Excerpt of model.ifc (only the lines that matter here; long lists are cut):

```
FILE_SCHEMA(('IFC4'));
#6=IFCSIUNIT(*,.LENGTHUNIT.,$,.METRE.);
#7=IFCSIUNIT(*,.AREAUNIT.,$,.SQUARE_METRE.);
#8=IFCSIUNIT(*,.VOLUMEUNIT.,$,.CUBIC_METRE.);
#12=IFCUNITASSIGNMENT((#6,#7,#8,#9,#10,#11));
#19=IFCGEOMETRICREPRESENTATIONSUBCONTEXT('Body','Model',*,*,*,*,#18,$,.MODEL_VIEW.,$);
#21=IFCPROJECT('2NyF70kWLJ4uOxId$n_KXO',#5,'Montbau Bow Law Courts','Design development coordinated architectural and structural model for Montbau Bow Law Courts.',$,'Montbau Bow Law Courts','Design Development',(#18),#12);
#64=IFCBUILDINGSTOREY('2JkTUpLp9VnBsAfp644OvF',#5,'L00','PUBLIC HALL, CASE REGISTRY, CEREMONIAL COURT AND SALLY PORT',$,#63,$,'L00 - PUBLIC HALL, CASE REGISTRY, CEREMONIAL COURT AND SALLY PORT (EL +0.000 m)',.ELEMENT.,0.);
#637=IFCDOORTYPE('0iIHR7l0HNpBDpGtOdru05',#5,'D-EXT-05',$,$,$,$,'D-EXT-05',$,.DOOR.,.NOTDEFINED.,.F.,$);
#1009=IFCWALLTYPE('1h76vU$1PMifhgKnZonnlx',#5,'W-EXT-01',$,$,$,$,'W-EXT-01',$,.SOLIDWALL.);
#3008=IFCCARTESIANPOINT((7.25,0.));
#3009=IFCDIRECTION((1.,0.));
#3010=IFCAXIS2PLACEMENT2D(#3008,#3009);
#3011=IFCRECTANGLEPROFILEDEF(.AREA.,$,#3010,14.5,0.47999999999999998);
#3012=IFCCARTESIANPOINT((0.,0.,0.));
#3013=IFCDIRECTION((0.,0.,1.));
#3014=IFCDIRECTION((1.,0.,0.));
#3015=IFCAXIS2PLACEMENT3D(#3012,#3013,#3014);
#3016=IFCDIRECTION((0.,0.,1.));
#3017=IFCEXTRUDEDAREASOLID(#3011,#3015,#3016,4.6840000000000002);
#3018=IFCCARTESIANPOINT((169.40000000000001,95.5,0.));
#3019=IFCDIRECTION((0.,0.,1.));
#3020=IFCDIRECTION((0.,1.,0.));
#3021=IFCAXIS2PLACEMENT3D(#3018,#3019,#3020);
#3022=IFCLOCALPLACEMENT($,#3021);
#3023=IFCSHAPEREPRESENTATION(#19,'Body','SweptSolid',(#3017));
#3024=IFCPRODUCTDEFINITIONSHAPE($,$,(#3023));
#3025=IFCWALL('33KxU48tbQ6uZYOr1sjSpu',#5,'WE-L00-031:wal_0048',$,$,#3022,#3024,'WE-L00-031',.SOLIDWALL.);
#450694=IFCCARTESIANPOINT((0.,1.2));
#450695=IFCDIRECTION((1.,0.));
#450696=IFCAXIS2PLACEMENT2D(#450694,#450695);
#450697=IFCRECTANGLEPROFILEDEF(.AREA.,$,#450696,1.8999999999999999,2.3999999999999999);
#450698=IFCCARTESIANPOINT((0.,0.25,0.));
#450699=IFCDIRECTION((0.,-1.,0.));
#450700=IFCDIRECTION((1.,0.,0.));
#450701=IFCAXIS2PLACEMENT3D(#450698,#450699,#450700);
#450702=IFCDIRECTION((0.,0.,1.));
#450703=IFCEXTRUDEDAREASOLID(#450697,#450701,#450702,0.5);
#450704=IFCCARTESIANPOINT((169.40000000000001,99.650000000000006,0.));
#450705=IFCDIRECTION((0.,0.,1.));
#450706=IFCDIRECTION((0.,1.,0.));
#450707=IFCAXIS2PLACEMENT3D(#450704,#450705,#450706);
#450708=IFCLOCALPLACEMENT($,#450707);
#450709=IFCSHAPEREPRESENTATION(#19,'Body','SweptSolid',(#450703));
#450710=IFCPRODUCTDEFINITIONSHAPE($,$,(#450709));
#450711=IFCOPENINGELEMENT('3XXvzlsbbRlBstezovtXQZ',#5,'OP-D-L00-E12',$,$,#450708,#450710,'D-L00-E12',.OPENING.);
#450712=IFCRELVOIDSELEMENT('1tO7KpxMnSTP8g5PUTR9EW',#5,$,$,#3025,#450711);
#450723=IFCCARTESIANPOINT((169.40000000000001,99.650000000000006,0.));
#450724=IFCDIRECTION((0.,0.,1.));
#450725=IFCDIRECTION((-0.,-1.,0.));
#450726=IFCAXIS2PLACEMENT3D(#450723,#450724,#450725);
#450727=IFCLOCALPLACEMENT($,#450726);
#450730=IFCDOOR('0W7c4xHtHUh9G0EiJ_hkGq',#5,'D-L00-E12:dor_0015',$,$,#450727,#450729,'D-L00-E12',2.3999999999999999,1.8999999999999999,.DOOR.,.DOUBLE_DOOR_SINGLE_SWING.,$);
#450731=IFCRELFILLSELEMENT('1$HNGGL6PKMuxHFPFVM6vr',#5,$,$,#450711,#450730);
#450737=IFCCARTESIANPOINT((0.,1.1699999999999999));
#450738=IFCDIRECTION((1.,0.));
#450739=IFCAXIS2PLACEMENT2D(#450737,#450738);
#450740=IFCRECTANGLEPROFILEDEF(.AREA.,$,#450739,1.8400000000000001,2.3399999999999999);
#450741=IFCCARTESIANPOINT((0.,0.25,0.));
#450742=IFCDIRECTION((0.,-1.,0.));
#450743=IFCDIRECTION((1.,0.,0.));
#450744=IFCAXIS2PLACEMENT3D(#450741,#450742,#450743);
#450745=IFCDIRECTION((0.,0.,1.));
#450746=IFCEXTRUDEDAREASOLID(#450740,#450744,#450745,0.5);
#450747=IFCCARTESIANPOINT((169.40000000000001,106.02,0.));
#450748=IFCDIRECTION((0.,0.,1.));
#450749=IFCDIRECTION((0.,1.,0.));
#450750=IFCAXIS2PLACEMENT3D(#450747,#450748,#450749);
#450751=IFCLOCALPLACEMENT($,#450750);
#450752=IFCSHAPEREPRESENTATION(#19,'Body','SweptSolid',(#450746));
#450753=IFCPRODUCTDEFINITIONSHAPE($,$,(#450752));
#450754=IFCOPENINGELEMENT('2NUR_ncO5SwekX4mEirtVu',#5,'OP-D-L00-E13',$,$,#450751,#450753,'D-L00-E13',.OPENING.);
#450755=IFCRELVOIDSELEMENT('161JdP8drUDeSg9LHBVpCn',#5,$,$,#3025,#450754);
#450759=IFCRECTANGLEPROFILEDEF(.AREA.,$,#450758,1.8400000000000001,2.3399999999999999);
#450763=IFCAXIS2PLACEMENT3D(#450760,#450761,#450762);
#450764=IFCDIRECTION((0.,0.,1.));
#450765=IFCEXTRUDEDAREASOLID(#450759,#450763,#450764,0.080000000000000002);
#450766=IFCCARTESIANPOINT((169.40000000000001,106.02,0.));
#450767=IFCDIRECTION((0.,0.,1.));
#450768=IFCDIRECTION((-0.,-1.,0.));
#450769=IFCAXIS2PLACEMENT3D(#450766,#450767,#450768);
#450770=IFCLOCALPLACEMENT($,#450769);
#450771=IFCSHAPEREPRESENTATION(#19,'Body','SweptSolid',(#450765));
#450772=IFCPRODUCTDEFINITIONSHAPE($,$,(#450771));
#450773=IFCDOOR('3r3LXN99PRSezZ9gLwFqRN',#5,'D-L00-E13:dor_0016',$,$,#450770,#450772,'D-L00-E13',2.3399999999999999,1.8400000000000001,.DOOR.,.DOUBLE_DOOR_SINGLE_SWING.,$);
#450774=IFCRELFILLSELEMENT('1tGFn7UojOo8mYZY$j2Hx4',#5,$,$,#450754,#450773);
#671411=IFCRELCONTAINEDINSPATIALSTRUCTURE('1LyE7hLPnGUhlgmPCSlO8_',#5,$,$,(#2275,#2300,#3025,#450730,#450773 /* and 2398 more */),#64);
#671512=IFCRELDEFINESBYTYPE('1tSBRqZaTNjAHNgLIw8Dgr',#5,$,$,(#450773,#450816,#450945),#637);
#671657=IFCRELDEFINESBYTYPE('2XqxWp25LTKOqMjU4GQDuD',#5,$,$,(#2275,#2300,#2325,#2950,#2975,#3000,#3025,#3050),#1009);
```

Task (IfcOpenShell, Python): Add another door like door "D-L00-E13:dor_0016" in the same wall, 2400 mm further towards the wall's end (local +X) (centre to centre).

```python
import ifcopenshell
import ifcopenshell.api.feature
import ifcopenshell.api.geometry
import ifcopenshell.api.root
import ifcopenshell.geom
import ifcopenshell.util.element
import ifcopenshell.util.placement
import ifcopenshell.util.shape

model = ifcopenshell.open("model.ifc")
settings = ifcopenshell.geom.settings()


def volume(element):
    """Net volume in cubic metres, openings subtracted."""
    shape = ifcopenshell.geom.create_shape(settings, element)
    return ifcopenshell.util.shape.get_volume(shape.geometry)


def reuse_history(source, copy):
    """copy_class also copies each property set's owner history, people and application; keep the originals."""
    for rel in copy.IsDefinedBy:
        if rel.is_a("IfcRelDefinesByProperties") and (history := rel.RelatingPropertyDefinition.OwnerHistory):
            rel.RelatingPropertyDefinition.OwnerHistory = source.OwnerHistory
            ifcopenshell.util.element.remove_deep2(model, history)


door = model.by_guid("3r3LXN99PRSezZ9gLwFqRN")
opening = door.FillsVoids[0].RelatingOpeningElement
wall = opening.VoidsElements[0].RelatingBuildingElement
before = volume(wall)
shift = ifcopenshell.util.placement.get_local_placement(wall.ObjectPlacement)[:3, 0] * 2.4

# copy_class copies the void relationship, type, container and properties, but no geometry.
new_opening = ifcopenshell.api.root.copy_class(model, product=opening)
new_opening.Representation = ifcopenshell.util.element.copy_deep(
    model, opening.Representation, exclude=["IfcGeometricRepresentationContext", "IfcRepresentationMap"]
)
new_opening.Tag = None
new_door = ifcopenshell.api.root.copy_class(model, product=door)
new_door.Representation = ifcopenshell.util.element.copy_deep(
    model, door.Representation, exclude=["IfcGeometricRepresentationContext", "IfcRepresentationMap"]
)
new_door.Tag = None
reuse_history(door, new_door)
ifcopenshell.api.feature.add_filling(model, opening=new_opening, element=new_door)

for old, new in ((opening, new_opening), (door, new_door)):
    matrix = ifcopenshell.util.placement.get_local_placement(old.ObjectPlacement)
    matrix[:3, 3] += shift
    ifcopenshell.api.geometry.edit_object_placement(model, product=new, matrix=matrix, is_si=False)

after = volume(wall)

print(f"wall volume {before:.3f} -> {after:.3f} m3")

model.write("model_rev.ifc")
```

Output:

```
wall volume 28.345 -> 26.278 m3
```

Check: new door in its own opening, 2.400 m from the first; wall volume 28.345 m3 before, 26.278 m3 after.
